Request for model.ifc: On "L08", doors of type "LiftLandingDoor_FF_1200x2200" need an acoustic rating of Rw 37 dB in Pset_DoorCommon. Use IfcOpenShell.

First a look at what the model holds.

```python
import ifcopenshell
import ifcopenshell.util.element

model = ifcopenshell.open("model.ifc")
print(model.schema)
storey = next(s for s in model.by_type("IfcBuildingStorey") if s.Name == "L08")
doors = [e for e in ifcopenshell.util.element.get_decomposition(storey) if e.is_a("IfcDoor")]
seen = {}
for e in doors:
    element_type = ifcopenshell.util.element.get_type(e)
    key = (element_type.Name if element_type != e and element_type else None, ifcopenshell.util.element.get_pset(e, "Pset_DoorCommon", "AcousticRating"))
    seen[key] = seen.get(key, 0) + 1
for (name, value), count in sorted(seen.items(), key=str):
    print(count, "x", name, "|", value)
```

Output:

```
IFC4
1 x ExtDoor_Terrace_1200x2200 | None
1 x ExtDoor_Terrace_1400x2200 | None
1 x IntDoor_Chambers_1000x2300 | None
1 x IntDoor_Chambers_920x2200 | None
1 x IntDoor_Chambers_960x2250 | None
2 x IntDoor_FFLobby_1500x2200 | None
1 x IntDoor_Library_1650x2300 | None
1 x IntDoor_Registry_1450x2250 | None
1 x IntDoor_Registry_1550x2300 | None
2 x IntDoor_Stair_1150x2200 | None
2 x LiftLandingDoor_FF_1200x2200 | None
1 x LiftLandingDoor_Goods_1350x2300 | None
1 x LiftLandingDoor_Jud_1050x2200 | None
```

```python
import ifcopenshell
import ifcopenshell.api.pset
import ifcopenshell.util.element

model = ifcopenshell.open("model.ifc")

storey = next(s for s in model.by_type("IfcBuildingStorey") if s.Name == "L08")
doors = [e for e in ifcopenshell.util.element.get_decomposition(storey) if e.is_a("IfcDoor")]

count = 0
for e in doors:
    element_type = ifcopenshell.util.element.get_type(e)
    if element_type in (None, e) or element_type.Name != "LiftLandingDoor_FF_1200x2200":
        continue
    # add_pset returns the element's existing set when there is one.
    pset = ifcopenshell.api.pset.add_pset(model, product=e, name="Pset_DoorCommon")
    ifcopenshell.api.pset.edit_pset(model, pset=pset, properties={"AcousticRating": "Rw 37 dB"})
    count += 1

print(count, "doors updated")

model.write("model_rev.ifc")
```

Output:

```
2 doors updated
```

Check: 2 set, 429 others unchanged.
